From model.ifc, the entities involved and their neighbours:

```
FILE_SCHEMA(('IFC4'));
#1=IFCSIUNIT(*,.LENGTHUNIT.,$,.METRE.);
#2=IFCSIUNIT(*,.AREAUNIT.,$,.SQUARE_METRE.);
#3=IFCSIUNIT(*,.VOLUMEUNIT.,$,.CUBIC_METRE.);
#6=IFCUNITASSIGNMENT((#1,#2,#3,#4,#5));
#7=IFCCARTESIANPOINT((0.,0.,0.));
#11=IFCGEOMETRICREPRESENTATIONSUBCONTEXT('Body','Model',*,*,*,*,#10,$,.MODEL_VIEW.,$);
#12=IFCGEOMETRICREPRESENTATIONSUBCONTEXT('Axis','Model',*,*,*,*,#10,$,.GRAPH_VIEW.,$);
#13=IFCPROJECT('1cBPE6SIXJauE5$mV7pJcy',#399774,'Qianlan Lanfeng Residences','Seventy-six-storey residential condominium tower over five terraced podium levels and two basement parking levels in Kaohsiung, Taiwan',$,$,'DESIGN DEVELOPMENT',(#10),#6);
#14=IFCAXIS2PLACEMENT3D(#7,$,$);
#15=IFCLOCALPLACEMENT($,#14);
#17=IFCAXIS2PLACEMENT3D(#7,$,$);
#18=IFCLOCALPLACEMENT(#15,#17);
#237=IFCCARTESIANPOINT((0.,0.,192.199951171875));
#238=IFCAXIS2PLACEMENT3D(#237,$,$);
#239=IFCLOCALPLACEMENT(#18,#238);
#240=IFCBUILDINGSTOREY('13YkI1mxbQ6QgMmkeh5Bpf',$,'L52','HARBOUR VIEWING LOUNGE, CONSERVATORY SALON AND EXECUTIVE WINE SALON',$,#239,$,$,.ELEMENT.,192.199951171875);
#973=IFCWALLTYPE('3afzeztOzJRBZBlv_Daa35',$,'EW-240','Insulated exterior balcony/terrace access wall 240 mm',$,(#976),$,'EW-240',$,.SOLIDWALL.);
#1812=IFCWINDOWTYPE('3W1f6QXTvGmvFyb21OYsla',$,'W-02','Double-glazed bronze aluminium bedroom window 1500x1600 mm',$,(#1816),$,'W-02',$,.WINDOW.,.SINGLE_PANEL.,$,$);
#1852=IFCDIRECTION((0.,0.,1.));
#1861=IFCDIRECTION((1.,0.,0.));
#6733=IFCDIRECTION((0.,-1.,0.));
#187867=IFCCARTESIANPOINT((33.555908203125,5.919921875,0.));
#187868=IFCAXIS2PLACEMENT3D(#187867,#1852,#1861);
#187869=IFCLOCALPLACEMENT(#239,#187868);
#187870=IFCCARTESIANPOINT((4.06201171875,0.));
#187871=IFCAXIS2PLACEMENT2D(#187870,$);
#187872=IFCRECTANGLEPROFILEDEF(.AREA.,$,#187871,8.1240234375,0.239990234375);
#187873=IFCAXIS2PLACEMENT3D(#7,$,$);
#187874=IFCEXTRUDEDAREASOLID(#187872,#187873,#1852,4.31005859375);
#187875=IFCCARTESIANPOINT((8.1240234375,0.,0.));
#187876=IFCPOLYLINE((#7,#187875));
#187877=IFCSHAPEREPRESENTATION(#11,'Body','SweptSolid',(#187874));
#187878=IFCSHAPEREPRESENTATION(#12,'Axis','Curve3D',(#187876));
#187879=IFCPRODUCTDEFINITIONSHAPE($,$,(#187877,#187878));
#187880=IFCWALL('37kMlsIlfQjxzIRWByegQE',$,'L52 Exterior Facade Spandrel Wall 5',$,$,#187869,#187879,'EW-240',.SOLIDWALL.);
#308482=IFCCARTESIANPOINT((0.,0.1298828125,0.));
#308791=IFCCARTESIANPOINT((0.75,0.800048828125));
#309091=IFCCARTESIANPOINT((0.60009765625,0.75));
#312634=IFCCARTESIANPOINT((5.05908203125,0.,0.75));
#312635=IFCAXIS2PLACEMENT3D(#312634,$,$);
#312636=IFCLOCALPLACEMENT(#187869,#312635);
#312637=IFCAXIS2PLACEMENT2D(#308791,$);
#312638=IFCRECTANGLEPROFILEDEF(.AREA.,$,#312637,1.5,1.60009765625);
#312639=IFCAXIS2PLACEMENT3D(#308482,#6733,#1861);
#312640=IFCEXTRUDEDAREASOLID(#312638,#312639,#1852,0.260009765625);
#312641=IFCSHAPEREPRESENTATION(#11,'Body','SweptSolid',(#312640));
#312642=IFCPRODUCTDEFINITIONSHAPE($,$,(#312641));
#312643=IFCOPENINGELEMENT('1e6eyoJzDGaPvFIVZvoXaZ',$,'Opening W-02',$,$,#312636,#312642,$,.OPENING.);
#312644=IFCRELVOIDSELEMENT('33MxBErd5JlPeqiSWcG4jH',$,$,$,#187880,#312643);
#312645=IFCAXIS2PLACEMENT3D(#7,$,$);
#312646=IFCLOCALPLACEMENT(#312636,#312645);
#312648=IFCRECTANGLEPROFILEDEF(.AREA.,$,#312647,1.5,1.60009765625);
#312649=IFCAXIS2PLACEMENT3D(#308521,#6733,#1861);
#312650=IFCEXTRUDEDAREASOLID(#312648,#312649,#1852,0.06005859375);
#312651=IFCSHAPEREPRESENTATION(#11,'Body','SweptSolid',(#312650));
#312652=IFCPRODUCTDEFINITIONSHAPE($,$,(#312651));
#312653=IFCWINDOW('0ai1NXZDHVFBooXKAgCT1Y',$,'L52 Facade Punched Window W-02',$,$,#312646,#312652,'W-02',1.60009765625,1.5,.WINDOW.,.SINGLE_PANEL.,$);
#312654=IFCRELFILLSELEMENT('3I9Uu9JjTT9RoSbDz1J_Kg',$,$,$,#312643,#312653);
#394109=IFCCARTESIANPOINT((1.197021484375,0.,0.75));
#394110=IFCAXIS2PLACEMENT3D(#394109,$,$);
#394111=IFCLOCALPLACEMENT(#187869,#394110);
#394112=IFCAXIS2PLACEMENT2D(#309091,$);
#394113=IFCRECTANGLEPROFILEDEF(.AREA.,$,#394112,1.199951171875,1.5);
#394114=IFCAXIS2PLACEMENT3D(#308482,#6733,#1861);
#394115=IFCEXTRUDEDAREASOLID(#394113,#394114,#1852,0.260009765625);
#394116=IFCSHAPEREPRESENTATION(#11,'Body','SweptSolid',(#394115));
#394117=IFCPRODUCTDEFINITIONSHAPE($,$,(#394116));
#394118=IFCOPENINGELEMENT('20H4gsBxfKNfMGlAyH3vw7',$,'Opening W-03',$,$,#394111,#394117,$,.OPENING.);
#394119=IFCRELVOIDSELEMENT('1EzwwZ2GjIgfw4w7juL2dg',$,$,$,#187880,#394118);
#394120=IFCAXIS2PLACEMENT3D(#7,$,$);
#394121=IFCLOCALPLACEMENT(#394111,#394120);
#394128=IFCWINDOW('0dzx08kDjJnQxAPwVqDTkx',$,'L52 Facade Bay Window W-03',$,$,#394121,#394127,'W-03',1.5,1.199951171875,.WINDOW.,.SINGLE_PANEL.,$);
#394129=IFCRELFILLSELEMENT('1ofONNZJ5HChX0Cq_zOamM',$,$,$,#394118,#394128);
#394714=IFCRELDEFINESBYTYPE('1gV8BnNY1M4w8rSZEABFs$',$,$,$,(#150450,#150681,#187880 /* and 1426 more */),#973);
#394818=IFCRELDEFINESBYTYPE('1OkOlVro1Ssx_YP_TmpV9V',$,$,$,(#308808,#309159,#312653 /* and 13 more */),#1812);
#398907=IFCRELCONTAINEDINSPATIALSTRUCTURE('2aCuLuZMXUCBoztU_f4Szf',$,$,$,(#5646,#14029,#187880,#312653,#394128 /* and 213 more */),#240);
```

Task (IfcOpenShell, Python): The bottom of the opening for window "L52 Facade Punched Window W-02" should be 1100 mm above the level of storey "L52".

```python
import numpy as np
import ifcopenshell
import ifcopenshell.api.geometry
import ifcopenshell.geom
import ifcopenshell.util.element
import ifcopenshell.util.placement
import ifcopenshell.util.shape
import ifcopenshell.util.unit

model = ifcopenshell.open("model.ifc")
unit_scale = ifcopenshell.util.unit.calculate_unit_scale(model)

window = model.by_guid("0ai1NXZDHVFBooXKAgCT1Y")
opening = window.FillsVoids[0].RelatingOpeningElement
storey = ifcopenshell.util.element.get_container(window, ifc_class="IfcBuildingStorey")
level = ifcopenshell.util.placement.get_local_placement(storey.ObjectPlacement)[2, 3]

# The opening's origin need not be at the sill, so measure its lowest point.
shape = ifcopenshell.geom.create_shape(ifcopenshell.geom.settings(), opening)
bottom = ifcopenshell.util.shape.get_shape_bottom_elevation(shape, shape.geometry) / unit_scale
dz = level + 1.1 / unit_scale - bottom

shift = np.array([0.0, 0.0, dz])
# The window is placed relative to its opening, so it follows when the opening moves.
matrix = ifcopenshell.util.placement.get_local_placement(opening.ObjectPlacement)
matrix[:3, 3] += shift
ifcopenshell.api.geometry.edit_object_placement(
    model, product=opening, matrix=matrix, is_si=False, should_transform_children=True
)

print(f"moved by {dz * unit_scale:+.3f} m")

model.write("model_updated.ifc")
```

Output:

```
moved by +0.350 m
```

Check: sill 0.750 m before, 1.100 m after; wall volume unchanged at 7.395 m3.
